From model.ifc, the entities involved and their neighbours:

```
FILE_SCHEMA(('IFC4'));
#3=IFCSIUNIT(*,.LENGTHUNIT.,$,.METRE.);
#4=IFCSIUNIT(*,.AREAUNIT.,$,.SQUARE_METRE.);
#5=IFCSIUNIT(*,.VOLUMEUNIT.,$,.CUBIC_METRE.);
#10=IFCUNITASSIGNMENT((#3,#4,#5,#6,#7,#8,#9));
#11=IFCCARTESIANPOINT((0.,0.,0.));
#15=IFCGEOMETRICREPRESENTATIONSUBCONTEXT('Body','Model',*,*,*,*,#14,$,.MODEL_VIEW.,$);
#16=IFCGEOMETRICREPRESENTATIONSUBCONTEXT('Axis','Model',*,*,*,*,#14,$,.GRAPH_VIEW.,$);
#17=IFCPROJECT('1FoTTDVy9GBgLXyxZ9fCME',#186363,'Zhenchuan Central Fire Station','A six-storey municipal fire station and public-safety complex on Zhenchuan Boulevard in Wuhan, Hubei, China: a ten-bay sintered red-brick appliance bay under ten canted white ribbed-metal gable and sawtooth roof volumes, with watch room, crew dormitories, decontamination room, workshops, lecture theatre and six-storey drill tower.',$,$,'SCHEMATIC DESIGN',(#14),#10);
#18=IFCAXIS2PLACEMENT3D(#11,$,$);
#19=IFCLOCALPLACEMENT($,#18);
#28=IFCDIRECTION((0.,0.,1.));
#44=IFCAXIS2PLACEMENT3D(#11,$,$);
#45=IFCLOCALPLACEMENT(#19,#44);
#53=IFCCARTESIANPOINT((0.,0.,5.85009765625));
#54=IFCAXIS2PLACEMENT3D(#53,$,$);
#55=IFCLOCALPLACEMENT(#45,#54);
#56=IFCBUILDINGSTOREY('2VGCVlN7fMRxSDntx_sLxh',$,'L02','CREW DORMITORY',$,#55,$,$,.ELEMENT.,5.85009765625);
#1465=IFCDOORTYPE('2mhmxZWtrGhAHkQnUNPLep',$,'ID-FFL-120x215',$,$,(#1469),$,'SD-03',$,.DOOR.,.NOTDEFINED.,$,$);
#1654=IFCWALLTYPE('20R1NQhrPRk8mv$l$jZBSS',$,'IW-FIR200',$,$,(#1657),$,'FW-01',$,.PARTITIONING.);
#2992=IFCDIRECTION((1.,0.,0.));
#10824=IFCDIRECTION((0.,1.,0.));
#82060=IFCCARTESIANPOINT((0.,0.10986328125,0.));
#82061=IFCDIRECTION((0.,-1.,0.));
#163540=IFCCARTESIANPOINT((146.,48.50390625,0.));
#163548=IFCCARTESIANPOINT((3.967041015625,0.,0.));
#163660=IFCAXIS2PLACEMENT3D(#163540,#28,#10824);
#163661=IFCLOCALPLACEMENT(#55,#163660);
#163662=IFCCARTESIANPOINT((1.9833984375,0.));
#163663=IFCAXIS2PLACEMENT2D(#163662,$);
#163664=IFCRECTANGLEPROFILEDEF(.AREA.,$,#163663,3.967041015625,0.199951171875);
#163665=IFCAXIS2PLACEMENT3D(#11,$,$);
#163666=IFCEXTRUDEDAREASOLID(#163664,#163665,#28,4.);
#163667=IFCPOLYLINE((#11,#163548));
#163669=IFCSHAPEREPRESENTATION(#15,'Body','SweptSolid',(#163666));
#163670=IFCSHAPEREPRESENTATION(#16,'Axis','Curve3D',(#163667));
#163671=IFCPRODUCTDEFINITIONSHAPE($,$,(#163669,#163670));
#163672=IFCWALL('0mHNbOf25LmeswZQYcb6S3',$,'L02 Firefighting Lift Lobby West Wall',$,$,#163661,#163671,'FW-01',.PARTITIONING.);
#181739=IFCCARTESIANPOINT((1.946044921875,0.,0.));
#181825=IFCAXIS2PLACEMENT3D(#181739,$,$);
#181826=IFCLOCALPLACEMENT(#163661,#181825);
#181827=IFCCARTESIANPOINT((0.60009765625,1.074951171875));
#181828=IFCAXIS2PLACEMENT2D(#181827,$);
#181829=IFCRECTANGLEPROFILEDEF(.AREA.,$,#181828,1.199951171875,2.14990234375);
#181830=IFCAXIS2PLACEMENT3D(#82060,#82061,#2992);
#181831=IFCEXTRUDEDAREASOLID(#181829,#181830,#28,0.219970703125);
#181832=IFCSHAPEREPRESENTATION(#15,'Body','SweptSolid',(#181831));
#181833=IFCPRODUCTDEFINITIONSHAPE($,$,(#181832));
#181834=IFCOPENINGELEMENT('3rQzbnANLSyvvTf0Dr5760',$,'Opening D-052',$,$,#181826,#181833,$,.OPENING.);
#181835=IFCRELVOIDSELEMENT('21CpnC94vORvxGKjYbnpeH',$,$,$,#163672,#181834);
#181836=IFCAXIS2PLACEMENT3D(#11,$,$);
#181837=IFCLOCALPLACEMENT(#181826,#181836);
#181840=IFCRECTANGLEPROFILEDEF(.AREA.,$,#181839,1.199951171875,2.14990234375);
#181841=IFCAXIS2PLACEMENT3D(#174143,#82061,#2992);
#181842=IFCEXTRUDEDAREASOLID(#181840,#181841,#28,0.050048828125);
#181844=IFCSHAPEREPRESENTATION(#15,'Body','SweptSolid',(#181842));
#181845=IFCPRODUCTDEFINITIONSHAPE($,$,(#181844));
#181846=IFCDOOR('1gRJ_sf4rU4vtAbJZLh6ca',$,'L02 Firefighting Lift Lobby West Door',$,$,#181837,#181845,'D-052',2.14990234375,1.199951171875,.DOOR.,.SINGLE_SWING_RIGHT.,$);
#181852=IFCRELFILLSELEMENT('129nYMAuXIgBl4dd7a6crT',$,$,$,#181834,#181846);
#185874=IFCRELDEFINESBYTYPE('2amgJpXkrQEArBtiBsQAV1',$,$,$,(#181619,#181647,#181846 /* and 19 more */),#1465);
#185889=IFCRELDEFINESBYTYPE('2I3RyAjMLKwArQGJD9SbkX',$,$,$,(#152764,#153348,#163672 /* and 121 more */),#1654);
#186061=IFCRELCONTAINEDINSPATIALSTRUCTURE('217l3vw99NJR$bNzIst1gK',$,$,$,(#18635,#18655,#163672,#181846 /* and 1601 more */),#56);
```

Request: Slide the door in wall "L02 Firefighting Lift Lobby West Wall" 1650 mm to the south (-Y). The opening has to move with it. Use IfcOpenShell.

```python
import ifcopenshell
import ifcopenshell.api.geometry
import ifcopenshell.util.placement
import ifcopenshell.util.unit

model = ifcopenshell.open("model.ifc")
unit_scale = ifcopenshell.util.unit.calculate_unit_scale(model)

door = model.by_guid("1gRJ_sf4rU4vtAbJZLh6ca")
opening = door.FillsVoids[0].RelatingOpeningElement
wall = opening.VoidsElements[0].RelatingBuildingElement

wall_matrix = ifcopenshell.util.placement.get_local_placement(wall.ObjectPlacement)
shift = wall_matrix[:3, 0] * -1.65 / unit_scale
before = ifcopenshell.util.placement.get_local_placement(door.ObjectPlacement)[:3, 3].copy()

# The door is placed relative to its opening, so it follows when the opening moves.
matrix = ifcopenshell.util.placement.get_local_placement(opening.ObjectPlacement)
matrix[:3, 3] += shift
ifcopenshell.api.geometry.edit_object_placement(
    model, product=opening, matrix=matrix, is_si=False, should_transform_children=True
)

after = ifcopenshell.util.placement.get_local_placement(door.ObjectPlacement)[:3, 3]
print("door moved by", (after - before).round(3) + 0.0)

model.write("model_rev.ifc")
```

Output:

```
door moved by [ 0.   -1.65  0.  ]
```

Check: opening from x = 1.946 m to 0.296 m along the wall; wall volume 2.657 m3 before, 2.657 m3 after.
